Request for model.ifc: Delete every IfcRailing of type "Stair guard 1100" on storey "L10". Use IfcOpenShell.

First a look at what the model holds.

```python
import ifcopenshell
import ifcopenshell.util.element

model = ifcopenshell.open("model.ifc")
print(model.schema)
storey = next(s for s in model.by_type("IfcBuildingStorey") if s.Name == "L10")
railings = [e for e in ifcopenshell.util.element.get_decomposition(storey) if e.is_a("IfcRailing")]
seen = {}
for e in railings:
    element_type = ifcopenshell.util.element.get_type(e)
    name = element_type.Name if element_type not in (None, e) else None
    seen[name] = seen.get(name, 0) + 1
for name, count in sorted(seen.items(), key=str):
    print(count, "x", name)
```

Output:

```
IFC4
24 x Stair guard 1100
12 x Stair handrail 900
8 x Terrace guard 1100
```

```python
import ifcopenshell
import ifcopenshell.api.root
import ifcopenshell.util.element

model = ifcopenshell.open("model.ifc")

storey = next(s for s in model.by_type("IfcBuildingStorey") if s.Name == "L10")
railings = [e for e in ifcopenshell.util.element.get_decomposition(storey) if e.is_a("IfcRailing")]
targets = [e for e in railings if (t := ifcopenshell.util.element.get_type(e)) not in (None, e) and t.Name == "Stair guard 1100"]

for e in targets:
    ifcopenshell.api.root.remove_product(model, product=e)
print(len(targets), "removed")

model.write("model_edited.ifc")
```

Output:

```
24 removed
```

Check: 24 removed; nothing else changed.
